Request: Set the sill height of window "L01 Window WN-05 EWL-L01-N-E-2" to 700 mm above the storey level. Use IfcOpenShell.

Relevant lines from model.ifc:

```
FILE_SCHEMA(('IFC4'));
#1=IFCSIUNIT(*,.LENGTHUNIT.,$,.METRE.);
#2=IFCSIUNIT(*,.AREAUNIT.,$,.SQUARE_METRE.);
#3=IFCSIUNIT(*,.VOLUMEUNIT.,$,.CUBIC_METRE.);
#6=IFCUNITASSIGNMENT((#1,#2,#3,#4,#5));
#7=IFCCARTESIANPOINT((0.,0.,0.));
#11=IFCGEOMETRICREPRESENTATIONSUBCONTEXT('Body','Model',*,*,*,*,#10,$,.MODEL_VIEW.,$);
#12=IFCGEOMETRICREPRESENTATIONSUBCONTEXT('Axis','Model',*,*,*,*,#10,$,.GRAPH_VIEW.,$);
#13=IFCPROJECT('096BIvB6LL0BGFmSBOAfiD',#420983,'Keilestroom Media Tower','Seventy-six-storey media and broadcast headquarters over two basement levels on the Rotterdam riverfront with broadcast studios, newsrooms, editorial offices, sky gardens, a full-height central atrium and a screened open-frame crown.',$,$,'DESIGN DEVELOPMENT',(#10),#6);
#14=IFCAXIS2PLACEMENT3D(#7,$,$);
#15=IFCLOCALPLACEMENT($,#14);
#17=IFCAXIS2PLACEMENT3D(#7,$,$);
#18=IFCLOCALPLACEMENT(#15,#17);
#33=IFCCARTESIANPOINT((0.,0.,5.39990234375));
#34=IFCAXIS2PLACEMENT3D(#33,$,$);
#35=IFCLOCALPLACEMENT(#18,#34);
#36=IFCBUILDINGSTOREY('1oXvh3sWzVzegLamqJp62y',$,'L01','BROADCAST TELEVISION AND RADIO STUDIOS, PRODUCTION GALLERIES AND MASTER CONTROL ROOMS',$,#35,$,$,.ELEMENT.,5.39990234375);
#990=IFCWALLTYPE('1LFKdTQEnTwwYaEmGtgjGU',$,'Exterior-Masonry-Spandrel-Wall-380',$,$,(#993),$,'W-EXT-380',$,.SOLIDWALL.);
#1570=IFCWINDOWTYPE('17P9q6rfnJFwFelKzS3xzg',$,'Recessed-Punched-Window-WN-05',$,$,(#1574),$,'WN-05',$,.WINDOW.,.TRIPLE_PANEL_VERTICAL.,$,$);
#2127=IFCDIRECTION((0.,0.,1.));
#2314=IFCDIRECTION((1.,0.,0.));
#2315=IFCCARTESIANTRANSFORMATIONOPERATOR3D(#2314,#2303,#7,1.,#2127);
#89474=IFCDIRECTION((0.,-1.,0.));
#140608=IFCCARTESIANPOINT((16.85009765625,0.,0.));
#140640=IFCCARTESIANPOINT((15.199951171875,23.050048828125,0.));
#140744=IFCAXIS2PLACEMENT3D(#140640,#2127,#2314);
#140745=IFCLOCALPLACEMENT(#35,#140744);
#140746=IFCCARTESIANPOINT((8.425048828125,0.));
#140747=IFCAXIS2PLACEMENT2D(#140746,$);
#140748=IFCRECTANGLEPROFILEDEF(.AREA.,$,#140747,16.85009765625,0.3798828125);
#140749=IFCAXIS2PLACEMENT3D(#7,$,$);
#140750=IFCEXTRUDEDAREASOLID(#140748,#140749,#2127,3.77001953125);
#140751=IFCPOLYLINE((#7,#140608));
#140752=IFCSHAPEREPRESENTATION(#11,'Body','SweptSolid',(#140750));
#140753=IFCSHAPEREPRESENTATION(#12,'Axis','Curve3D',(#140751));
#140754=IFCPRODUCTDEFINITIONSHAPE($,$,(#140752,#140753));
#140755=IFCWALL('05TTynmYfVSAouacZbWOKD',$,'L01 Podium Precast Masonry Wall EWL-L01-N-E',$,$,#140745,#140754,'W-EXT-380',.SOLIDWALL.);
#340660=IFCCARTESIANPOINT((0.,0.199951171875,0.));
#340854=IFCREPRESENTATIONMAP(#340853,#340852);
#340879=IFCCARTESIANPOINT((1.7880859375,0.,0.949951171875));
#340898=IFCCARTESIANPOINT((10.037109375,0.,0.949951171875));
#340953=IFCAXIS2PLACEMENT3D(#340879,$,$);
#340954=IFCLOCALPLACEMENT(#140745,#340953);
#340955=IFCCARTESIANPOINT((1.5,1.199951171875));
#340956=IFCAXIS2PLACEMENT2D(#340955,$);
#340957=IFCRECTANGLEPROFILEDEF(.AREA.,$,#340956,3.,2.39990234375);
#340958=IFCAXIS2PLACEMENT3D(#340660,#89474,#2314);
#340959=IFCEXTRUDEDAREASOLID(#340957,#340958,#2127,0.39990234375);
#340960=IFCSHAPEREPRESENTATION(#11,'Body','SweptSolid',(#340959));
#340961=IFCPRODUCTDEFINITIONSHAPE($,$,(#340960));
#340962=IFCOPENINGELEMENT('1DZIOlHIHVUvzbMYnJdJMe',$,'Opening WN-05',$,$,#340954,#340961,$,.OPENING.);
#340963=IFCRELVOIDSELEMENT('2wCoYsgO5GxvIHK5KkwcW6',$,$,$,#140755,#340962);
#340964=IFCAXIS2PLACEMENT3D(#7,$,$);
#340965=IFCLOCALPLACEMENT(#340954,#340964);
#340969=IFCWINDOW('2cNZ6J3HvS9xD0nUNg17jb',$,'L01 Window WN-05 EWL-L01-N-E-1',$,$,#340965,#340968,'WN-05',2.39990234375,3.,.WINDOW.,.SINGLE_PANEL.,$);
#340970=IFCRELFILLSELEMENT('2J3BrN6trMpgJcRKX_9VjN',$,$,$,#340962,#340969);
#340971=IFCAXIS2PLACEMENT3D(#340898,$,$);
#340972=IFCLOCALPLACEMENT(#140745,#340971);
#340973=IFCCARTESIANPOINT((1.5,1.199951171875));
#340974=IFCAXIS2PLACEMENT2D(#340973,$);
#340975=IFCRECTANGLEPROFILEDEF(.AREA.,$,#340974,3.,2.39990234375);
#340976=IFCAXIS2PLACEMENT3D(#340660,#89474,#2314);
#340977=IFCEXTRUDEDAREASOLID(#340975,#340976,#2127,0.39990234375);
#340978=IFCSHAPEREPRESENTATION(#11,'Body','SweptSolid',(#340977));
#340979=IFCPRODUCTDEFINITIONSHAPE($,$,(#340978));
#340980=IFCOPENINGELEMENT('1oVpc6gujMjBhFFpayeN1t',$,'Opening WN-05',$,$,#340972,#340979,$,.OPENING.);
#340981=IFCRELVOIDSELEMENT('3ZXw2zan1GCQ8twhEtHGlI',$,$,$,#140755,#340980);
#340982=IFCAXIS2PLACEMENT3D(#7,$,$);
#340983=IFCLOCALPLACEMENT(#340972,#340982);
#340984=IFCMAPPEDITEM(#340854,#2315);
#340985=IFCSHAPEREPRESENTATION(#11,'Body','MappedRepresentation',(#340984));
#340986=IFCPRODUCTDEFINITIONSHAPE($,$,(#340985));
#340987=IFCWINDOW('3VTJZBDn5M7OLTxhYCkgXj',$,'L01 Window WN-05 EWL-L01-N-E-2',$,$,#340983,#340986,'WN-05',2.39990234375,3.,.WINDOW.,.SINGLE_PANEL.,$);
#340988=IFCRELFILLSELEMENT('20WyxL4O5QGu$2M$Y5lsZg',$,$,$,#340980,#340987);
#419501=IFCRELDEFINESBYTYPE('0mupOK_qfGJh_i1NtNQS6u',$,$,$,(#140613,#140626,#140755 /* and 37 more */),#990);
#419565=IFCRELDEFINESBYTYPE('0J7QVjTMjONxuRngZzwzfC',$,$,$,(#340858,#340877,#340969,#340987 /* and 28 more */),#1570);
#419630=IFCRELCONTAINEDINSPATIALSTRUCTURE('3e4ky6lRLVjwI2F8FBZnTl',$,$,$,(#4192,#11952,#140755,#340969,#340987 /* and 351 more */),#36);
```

```python
import numpy as np
import ifcopenshell
import ifcopenshell.api.geometry
import ifcopenshell.geom
import ifcopenshell.util.element
import ifcopenshell.util.placement
import ifcopenshell.util.shape
import ifcopenshell.util.unit

model = ifcopenshell.open("model.ifc")
unit_scale = ifcopenshell.util.unit.calculate_unit_scale(model)

window = model.by_guid("3VTJZBDn5M7OLTxhYCkgXj")
opening = window.FillsVoids[0].RelatingOpeningElement
storey = ifcopenshell.util.element.get_container(window, ifc_class="IfcBuildingStorey")
level = ifcopenshell.util.placement.get_local_placement(storey.ObjectPlacement)[2, 3]

# The opening's origin need not be at the sill, so measure its lowest point.
shape = ifcopenshell.geom.create_shape(ifcopenshell.geom.settings(), opening)
bottom = ifcopenshell.util.shape.get_shape_bottom_elevation(shape, shape.geometry) / unit_scale
dz = level + 0.7 / unit_scale - bottom

shift = np.array([0.0, 0.0, dz])
# The window is placed relative to its opening, so it follows when the opening moves.
matrix = ifcopenshell.util.placement.get_local_placement(opening.ObjectPlacement)
matrix[:3, 3] += shift
ifcopenshell.api.geometry.edit_object_placement(
    model, product=opening, matrix=matrix, is_si=False, should_transform_children=True
)

print(f"moved by {dz * unit_scale:+.3f} m")

model.write("model-out.ifc")
```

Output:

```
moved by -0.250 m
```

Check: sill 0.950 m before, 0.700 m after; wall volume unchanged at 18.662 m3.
